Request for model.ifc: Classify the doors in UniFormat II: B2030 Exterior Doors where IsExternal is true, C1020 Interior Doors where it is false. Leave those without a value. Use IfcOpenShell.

First a look at what the model holds.

```python
import ifcopenshell
import ifcopenshell.util.element

model = ifcopenshell.open("model.ifc")
print(model.schema)
print("classifications:", [c.Name for c in model.by_type("IfcClassification")])
values = [ifcopenshell.util.element.get_pset(e, "Pset_DoorCommon", "IsExternal") for e in model.by_type("IfcDoor")]
for value in (True, False, None):
    print("IsExternal", value, values.count(value))
```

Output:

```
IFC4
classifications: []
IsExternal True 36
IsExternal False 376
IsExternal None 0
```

```python
import ifcopenshell
import ifcopenshell.api.classification
import ifcopenshell.util.element

model = ifcopenshell.open("model.ifc")

system = ifcopenshell.api.classification.add_classification(model, classification="UniFormat II")

doors = model.by_type("IfcDoor")
external = {e: ifcopenshell.util.element.get_pset(e, "Pset_DoorCommon", "IsExternal") for e in doors}
for flag, code, name in ((True, "B2030", "Exterior Doors"), (False, "C1020", "Interior Doors")):
    products = [e for e in doors if external[e] is flag]
    ifcopenshell.api.classification.add_reference(
        model, products=products, classification=system, identification=code, name=name
    )
    print(code, len(products))

model.write("model_edited.ifc")
```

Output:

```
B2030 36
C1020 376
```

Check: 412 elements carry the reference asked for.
